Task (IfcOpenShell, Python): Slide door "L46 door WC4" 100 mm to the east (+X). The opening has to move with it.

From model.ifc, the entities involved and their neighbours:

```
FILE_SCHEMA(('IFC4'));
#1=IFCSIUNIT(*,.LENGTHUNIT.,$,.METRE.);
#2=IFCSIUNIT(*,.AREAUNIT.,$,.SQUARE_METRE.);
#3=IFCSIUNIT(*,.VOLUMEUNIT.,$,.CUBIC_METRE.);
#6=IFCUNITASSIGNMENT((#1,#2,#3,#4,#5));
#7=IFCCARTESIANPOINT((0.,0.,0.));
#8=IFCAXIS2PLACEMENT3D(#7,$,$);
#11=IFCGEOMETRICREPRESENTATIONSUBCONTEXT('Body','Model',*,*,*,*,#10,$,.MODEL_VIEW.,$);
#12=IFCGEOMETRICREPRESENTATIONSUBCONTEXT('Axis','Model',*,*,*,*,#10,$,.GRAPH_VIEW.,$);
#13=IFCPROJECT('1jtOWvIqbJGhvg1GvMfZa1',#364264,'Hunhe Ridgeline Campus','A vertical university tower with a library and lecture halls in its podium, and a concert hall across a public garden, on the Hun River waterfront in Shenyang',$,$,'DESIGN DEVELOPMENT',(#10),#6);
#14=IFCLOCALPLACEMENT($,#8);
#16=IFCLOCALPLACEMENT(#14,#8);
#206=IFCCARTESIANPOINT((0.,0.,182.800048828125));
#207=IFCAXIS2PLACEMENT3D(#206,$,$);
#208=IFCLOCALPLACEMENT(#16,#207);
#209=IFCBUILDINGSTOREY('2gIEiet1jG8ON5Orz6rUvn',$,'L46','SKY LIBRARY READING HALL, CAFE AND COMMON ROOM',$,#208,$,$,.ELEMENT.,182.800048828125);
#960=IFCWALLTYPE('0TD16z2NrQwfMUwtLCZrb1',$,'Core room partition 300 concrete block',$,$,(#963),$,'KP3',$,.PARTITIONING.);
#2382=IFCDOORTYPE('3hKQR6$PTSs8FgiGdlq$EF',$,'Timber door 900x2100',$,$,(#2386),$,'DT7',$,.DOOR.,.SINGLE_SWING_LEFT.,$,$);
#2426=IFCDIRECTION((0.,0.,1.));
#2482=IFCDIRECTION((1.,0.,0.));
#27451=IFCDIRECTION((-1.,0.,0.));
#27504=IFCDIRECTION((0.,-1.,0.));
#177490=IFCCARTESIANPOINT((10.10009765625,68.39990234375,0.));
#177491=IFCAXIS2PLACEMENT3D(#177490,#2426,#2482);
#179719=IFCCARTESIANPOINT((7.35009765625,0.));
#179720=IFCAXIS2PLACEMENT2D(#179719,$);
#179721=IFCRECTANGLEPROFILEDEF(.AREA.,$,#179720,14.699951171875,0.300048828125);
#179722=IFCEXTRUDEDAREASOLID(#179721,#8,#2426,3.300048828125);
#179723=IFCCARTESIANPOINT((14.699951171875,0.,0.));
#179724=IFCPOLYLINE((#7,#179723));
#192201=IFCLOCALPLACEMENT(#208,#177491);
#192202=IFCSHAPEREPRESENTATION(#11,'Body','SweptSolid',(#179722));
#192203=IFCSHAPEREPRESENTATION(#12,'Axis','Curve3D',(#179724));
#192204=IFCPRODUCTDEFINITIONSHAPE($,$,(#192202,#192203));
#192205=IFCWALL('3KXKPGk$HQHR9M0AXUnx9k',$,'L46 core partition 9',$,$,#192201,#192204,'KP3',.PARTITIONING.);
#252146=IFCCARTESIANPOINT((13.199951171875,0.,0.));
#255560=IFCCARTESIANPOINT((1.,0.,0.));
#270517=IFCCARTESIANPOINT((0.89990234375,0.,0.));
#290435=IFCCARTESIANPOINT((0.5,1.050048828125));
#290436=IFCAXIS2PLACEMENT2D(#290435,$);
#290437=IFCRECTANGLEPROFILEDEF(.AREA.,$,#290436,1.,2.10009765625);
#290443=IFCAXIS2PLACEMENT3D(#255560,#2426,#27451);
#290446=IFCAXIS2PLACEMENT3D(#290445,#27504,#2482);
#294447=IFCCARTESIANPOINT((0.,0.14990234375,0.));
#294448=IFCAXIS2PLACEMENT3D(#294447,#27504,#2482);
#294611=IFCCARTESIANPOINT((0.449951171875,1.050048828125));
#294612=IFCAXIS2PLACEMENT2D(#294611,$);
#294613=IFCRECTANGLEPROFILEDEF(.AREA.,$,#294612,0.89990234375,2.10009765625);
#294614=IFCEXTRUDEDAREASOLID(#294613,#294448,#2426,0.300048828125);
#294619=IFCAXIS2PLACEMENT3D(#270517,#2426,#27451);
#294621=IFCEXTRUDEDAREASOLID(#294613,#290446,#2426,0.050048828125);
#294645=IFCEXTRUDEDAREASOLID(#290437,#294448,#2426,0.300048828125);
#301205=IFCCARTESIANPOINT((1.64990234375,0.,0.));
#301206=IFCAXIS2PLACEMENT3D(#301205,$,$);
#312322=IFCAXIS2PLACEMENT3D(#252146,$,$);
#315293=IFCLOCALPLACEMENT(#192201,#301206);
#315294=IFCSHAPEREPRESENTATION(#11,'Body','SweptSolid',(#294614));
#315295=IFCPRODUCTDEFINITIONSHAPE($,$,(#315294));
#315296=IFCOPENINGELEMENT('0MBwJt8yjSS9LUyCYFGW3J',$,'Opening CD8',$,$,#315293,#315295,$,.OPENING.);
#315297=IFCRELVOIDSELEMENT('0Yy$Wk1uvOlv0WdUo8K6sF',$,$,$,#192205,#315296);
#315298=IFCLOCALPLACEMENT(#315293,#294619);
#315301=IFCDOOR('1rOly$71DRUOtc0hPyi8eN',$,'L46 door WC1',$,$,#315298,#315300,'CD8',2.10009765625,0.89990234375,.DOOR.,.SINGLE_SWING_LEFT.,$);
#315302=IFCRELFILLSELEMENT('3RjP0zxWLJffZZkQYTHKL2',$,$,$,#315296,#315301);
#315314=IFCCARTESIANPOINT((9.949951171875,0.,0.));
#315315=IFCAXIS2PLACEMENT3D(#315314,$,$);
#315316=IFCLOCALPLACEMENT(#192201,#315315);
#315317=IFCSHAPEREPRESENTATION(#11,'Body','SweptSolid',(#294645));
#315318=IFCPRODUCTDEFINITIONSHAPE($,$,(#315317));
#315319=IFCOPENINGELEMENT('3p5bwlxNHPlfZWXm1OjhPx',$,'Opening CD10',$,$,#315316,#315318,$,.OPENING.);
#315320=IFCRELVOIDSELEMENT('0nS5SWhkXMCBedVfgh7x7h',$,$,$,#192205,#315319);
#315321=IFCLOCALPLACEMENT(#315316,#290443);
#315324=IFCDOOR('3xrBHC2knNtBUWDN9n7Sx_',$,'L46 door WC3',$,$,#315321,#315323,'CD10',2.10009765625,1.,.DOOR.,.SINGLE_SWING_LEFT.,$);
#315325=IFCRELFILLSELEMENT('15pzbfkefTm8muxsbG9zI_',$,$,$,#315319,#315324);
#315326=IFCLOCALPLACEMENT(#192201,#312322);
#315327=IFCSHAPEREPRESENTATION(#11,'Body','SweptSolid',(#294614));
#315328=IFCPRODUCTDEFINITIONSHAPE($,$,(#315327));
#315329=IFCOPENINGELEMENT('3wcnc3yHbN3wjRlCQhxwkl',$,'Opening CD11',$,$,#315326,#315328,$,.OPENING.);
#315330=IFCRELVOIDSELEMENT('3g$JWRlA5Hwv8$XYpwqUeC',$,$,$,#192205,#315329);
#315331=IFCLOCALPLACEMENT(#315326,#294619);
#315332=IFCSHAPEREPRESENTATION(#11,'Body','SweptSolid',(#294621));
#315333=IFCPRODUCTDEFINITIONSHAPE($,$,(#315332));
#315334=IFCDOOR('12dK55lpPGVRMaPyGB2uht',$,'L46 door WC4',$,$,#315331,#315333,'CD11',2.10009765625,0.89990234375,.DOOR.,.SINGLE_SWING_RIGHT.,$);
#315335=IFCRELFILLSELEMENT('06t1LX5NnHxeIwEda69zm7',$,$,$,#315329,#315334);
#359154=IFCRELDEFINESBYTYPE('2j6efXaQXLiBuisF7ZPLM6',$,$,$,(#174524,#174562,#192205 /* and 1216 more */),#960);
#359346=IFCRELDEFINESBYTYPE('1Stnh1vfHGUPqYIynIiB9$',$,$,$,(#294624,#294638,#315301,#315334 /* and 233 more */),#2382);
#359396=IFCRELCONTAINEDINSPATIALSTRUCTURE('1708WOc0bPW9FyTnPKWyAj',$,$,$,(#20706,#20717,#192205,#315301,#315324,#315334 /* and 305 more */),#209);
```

```python
import ifcopenshell
import ifcopenshell.api.geometry
import ifcopenshell.util.placement
import ifcopenshell.util.unit

model = ifcopenshell.open("model.ifc")
unit_scale = ifcopenshell.util.unit.calculate_unit_scale(model)

door = model.by_id(315334)
opening = door.FillsVoids[0].RelatingOpeningElement
wall = opening.VoidsElements[0].RelatingBuildingElement

wall_matrix = ifcopenshell.util.placement.get_local_placement(wall.ObjectPlacement)
shift = wall_matrix[:3, 0] * 0.1 / unit_scale
before = ifcopenshell.util.placement.get_local_placement(door.ObjectPlacement)[:3, 3].copy()

# The door is placed relative to its opening, so it follows when the opening moves.
matrix = ifcopenshell.util.placement.get_local_placement(opening.ObjectPlacement)
matrix[:3, 3] += shift
ifcopenshell.api.geometry.edit_object_placement(
    model, product=opening, matrix=matrix, is_si=False, should_transform_children=True
)

after = ifcopenshell.util.placement.get_local_placement(door.ObjectPlacement)[:3, 3]
print("door moved by", (after - before).round(3) + 0.0)

model.write("model-out.ifc")
```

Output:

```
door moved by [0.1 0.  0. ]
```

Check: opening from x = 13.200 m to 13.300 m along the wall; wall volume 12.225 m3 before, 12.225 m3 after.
